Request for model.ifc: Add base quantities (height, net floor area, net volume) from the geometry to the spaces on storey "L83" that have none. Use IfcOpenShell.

First a look at what the model holds.

```python
import ifcopenshell
import ifcopenshell.util.element
import ifcopenshell.util.unit

model = ifcopenshell.open("model.ifc")
print(model.schema)
for unit_type in ("LENGTHUNIT", "AREAUNIT", "VOLUMEUNIT"):
    print(unit_type, ifcopenshell.util.unit.calculate_unit_scale(model, unit_type))
storey = next(s for s in model.by_type("IfcBuildingStorey") if s.Name == "L83")
spaces = [e for e in ifcopenshell.util.element.get_decomposition(storey) if e.is_a("IfcSpace")]
for e in sorted(spaces, key=lambda e: e.id()):
    print(e.id(), e.is_a(), e.Name, list(ifcopenshell.util.element.get_psets(e, qtos_only=True)), sep=" | ")
```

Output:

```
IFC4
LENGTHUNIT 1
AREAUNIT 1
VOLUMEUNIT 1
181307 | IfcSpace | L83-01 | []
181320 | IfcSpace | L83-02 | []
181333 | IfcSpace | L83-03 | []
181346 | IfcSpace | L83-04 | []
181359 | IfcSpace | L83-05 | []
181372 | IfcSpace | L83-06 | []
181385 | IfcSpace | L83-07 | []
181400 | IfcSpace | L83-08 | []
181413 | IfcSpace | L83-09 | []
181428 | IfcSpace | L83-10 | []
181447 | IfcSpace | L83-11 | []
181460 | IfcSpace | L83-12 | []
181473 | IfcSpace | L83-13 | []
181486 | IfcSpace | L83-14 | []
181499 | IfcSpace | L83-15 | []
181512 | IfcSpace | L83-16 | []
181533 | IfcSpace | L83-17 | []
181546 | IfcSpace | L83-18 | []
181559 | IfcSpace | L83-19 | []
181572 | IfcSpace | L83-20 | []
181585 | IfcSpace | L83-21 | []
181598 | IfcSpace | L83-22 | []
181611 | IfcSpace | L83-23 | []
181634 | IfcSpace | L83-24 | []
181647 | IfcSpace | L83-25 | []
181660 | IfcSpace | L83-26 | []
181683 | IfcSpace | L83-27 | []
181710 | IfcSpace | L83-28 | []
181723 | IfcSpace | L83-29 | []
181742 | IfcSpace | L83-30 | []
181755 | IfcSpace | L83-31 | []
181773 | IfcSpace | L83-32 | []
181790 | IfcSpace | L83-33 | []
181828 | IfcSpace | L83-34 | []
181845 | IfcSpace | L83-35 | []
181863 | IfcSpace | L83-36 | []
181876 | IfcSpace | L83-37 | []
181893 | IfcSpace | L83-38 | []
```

```python
import ifcopenshell
import ifcopenshell.api.pset
import ifcopenshell.geom
import ifcopenshell.util.element
import ifcopenshell.util.shape
import ifcopenshell.util.unit

model = ifcopenshell.open("model.ifc")
unit_scale = ifcopenshell.util.unit.calculate_unit_scale(model)
area_scale = ifcopenshell.util.unit.calculate_unit_scale(model, "AREAUNIT")
volume_scale = ifcopenshell.util.unit.calculate_unit_scale(model, "VOLUMEUNIT")
settings = ifcopenshell.geom.settings()

storey = next(s for s in model.by_type("IfcBuildingStorey") if s.Name == "L83")
spaces = [e for e in ifcopenshell.util.element.get_decomposition(storey) if e.is_a("IfcSpace")]

for e in sorted(spaces, key=lambda e: e.id()):
    if ifcopenshell.util.element.get_psets(e, qtos_only=True, should_inherit=False):
        continue
    # Geometry comes back in metres, in the element's own axes.
    shape = ifcopenshell.geom.create_shape(settings, e)
    values = {
        "Height": ifcopenshell.util.shape.get_z(shape.geometry) / unit_scale,
        "NetFloorArea": ifcopenshell.util.shape.get_footprint_area(shape.geometry) / area_scale,
        "NetVolume": ifcopenshell.util.shape.get_volume(shape.geometry) / volume_scale,
    }
    qto = ifcopenshell.api.pset.add_qto(model, product=e, name="Qto_SpaceBaseQuantities")
    ifcopenshell.api.pset.edit_qto(model, qto=qto, properties=values)
    print(e.id(), {k: round(v, 3) for k, v in values.items()})

model.write("model-out.ifc")
```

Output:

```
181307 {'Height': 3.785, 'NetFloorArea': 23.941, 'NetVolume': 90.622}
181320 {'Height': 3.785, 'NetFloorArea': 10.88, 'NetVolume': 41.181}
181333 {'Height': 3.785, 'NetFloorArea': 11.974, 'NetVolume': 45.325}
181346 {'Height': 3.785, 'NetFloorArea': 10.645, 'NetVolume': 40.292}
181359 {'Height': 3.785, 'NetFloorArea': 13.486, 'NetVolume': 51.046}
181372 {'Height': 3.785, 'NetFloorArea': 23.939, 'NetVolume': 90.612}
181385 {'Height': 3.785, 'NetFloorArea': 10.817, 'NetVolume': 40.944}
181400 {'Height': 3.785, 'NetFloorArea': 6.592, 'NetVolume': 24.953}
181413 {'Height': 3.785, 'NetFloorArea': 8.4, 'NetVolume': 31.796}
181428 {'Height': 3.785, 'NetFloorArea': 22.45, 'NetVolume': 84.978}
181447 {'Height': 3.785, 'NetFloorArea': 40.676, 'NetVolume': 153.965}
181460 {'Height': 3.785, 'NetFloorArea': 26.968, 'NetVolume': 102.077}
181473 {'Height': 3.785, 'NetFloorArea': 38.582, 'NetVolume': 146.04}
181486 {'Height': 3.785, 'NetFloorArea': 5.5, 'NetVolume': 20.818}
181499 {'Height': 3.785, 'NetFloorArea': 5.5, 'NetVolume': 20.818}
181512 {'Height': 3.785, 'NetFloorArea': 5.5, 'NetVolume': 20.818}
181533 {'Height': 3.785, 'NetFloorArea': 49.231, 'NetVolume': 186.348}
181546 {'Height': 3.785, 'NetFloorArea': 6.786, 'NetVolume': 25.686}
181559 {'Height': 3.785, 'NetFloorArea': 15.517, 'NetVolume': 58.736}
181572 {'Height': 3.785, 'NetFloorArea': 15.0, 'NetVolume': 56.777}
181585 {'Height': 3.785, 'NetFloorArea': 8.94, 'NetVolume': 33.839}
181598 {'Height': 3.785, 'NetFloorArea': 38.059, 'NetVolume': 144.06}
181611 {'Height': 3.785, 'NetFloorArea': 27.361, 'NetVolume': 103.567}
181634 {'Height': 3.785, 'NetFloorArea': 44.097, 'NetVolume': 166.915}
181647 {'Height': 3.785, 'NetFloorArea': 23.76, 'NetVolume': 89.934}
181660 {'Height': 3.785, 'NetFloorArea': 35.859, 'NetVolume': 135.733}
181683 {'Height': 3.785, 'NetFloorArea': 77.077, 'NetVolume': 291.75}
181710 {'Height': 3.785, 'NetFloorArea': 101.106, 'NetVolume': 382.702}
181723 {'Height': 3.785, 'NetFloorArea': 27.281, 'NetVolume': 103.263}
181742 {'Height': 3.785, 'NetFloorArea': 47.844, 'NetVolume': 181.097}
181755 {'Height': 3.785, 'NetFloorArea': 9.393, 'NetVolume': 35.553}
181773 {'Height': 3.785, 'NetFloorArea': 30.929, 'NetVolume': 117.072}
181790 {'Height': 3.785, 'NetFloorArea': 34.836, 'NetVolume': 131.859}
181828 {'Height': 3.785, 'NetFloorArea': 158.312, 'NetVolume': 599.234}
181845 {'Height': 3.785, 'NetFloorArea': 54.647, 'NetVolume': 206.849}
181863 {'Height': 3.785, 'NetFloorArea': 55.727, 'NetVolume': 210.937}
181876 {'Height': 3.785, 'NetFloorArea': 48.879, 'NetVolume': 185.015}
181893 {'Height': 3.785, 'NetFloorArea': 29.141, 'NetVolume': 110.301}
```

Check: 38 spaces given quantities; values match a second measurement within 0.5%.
